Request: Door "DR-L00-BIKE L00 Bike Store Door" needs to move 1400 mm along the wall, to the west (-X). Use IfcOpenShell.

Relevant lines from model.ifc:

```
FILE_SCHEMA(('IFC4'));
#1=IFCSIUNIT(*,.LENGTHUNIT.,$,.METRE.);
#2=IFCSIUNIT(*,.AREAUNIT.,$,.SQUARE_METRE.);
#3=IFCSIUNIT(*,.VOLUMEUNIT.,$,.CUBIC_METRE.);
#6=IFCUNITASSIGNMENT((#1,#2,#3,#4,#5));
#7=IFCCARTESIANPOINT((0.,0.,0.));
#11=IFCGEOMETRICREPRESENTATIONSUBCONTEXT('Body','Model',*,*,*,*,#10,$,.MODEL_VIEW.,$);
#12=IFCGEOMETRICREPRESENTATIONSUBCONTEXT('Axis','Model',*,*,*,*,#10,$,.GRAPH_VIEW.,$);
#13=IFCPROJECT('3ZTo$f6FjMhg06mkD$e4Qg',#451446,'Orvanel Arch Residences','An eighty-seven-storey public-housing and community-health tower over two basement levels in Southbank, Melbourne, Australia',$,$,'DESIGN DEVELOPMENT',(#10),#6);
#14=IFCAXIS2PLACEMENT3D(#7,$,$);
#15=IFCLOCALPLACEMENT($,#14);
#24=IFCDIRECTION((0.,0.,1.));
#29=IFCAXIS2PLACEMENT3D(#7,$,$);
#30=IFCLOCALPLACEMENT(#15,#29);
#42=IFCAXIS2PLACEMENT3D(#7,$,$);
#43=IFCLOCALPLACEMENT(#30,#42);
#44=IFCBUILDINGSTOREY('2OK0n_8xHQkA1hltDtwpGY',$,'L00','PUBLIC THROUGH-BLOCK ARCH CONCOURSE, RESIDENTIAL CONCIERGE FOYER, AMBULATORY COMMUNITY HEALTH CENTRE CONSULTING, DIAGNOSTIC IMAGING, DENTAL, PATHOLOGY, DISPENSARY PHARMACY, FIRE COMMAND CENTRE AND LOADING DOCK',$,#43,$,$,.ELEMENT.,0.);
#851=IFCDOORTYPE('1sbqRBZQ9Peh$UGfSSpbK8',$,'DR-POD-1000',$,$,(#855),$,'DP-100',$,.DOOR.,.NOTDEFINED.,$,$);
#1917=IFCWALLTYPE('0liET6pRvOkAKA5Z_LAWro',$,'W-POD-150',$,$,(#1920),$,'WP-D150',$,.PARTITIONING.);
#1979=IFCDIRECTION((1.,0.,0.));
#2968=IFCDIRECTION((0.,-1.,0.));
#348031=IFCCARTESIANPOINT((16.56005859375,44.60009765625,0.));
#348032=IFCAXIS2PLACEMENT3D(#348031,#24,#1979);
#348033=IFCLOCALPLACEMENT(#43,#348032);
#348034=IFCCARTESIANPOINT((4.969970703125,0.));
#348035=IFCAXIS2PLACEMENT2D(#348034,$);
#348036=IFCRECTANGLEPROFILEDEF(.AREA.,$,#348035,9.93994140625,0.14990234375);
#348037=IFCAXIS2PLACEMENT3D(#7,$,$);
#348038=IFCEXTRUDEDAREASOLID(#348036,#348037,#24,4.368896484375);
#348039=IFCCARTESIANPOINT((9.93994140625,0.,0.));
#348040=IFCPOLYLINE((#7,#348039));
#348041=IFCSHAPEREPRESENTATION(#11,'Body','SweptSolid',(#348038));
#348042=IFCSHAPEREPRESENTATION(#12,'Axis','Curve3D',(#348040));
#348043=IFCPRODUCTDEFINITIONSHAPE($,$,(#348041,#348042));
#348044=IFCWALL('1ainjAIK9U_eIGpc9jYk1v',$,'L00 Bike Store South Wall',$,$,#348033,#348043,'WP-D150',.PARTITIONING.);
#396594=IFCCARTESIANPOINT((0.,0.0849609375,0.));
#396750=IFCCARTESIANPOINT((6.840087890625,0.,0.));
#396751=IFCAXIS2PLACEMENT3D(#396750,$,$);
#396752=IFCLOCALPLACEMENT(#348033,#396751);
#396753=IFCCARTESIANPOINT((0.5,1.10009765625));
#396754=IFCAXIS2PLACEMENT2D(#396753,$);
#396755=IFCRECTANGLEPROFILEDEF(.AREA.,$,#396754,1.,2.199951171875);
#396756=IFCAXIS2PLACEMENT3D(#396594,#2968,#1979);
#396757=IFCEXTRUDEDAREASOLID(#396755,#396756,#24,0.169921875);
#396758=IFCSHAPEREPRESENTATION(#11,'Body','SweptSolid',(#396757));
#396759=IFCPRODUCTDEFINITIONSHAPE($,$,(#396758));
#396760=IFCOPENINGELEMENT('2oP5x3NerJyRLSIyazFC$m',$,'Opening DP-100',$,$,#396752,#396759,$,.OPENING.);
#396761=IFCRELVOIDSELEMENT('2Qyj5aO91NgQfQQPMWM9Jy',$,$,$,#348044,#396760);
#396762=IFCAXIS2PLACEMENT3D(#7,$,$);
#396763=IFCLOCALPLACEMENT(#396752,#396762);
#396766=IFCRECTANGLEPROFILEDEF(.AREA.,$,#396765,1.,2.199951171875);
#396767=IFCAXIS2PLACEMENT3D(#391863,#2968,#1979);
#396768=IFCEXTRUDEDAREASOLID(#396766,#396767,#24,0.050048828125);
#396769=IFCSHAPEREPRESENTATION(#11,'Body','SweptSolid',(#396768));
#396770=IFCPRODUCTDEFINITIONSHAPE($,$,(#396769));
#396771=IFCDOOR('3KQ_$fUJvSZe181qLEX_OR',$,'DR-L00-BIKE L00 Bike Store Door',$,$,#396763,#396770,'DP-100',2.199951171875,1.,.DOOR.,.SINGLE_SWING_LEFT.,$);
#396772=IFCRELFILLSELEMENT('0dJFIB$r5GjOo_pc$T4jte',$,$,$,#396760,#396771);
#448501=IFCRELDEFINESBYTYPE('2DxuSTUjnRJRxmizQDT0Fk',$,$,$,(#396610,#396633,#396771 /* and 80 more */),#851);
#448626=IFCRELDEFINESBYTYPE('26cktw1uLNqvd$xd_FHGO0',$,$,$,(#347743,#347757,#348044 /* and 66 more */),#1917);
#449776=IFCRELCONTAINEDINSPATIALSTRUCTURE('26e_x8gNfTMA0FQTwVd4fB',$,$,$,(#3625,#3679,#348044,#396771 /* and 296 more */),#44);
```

```python
import ifcopenshell
import ifcopenshell.api.geometry
import ifcopenshell.util.placement
import ifcopenshell.util.unit

model = ifcopenshell.open("model.ifc")
unit_scale = ifcopenshell.util.unit.calculate_unit_scale(model)

door = model.by_id(396771)
opening = door.FillsVoids[0].RelatingOpeningElement
wall = opening.VoidsElements[0].RelatingBuildingElement

wall_matrix = ifcopenshell.util.placement.get_local_placement(wall.ObjectPlacement)
shift = wall_matrix[:3, 0] * -1.4 / unit_scale
before = ifcopenshell.util.placement.get_local_placement(door.ObjectPlacement)[:3, 3].copy()

# The door is placed relative to its opening, so it follows when the opening moves.
matrix = ifcopenshell.util.placement.get_local_placement(opening.ObjectPlacement)
matrix[:3, 3] += shift
ifcopenshell.api.geometry.edit_object_placement(
    model, product=opening, matrix=matrix, is_si=False, should_transform_children=True
)

after = ifcopenshell.util.placement.get_local_placement(door.ObjectPlacement)[:3, 3]
print("door moved by", (after - before).round(3) + 0.0)

model.write("model_v2.ifc")
```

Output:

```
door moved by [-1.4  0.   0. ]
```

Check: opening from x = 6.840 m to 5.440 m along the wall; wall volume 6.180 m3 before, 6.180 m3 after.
